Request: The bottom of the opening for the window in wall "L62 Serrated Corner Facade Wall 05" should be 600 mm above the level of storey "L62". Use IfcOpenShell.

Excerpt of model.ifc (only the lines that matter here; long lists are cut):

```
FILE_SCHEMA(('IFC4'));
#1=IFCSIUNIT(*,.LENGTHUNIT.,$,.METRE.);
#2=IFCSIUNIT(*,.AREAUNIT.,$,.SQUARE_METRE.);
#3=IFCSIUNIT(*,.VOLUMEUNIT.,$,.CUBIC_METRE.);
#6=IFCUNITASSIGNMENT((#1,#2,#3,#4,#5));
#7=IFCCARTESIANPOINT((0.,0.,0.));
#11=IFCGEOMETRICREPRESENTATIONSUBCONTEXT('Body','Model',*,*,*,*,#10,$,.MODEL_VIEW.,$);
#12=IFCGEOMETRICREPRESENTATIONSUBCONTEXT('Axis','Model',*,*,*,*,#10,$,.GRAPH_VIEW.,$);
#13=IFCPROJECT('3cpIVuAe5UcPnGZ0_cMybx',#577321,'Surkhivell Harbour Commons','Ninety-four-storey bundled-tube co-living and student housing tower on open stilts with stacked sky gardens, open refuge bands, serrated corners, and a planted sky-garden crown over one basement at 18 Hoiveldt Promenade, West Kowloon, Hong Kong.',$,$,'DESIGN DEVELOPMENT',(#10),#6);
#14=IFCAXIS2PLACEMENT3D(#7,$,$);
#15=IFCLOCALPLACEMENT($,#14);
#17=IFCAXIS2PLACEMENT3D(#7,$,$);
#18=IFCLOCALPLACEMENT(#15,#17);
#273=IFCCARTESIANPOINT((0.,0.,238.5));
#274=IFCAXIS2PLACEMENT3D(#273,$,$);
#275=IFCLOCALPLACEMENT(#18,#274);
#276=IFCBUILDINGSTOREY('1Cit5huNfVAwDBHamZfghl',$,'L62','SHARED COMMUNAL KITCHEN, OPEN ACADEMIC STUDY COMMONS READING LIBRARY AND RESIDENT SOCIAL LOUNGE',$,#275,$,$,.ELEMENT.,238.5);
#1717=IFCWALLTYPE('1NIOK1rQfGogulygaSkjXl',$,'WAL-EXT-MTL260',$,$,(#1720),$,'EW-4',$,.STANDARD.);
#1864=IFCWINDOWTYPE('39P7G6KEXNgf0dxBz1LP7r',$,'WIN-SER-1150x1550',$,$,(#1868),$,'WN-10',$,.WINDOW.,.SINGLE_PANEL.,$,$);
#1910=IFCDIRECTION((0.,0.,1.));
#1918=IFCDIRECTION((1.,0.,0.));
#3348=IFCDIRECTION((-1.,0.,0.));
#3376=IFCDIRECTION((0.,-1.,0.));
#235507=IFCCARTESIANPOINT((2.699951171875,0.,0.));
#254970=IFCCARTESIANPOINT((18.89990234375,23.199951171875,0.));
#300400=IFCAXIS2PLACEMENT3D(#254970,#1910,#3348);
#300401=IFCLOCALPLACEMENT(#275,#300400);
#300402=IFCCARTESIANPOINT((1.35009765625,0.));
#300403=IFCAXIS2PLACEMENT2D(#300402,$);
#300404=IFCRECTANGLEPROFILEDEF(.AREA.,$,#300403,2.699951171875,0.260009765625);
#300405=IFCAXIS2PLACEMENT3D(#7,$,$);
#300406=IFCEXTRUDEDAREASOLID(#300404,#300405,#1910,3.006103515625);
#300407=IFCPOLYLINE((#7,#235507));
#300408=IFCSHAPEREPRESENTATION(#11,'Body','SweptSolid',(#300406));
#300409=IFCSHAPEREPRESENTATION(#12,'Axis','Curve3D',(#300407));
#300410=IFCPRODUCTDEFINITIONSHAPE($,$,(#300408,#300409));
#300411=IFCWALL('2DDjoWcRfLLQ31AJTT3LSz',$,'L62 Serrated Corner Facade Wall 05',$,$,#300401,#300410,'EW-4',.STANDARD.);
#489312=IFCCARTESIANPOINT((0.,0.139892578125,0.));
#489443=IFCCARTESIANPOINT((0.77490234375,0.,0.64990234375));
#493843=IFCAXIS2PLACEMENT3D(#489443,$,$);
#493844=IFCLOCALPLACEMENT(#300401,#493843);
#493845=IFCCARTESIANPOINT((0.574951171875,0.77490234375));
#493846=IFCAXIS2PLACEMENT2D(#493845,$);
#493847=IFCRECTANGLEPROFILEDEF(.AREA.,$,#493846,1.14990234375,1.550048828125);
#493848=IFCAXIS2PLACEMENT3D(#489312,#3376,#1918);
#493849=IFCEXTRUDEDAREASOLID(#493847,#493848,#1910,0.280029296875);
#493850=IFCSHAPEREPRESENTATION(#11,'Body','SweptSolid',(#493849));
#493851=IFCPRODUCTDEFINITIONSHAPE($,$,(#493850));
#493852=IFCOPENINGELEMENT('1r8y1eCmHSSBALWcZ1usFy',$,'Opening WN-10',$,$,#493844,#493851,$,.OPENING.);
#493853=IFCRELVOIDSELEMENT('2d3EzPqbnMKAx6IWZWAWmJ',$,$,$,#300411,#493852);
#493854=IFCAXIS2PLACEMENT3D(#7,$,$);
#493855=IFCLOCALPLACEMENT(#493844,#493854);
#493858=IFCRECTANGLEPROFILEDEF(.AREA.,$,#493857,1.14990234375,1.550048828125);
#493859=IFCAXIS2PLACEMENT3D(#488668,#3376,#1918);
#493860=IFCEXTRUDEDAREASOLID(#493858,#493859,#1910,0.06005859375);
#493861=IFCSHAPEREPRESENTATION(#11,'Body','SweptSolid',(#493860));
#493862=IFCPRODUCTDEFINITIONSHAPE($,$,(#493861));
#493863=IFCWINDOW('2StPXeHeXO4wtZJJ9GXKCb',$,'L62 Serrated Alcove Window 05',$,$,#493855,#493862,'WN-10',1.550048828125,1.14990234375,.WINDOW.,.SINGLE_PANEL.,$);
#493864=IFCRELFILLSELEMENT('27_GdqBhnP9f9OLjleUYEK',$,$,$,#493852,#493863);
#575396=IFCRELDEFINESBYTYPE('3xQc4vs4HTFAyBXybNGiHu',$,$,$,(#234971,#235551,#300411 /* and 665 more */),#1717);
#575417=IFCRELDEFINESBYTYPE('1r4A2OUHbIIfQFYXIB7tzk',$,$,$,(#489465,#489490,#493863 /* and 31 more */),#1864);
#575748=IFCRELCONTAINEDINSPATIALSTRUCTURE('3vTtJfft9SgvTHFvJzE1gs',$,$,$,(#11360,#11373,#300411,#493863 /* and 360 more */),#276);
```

```python
import numpy as np
import ifcopenshell
import ifcopenshell.api.geometry
import ifcopenshell.geom
import ifcopenshell.util.element
import ifcopenshell.util.placement
import ifcopenshell.util.shape
import ifcopenshell.util.unit

model = ifcopenshell.open("model.ifc")
unit_scale = ifcopenshell.util.unit.calculate_unit_scale(model)

window = model.by_guid("2StPXeHeXO4wtZJJ9GXKCb")
opening = window.FillsVoids[0].RelatingOpeningElement
storey = ifcopenshell.util.element.get_container(window, ifc_class="IfcBuildingStorey")
level = ifcopenshell.util.placement.get_local_placement(storey.ObjectPlacement)[2, 3]

# The opening's origin need not be at the sill, so measure its lowest point.
shape = ifcopenshell.geom.create_shape(ifcopenshell.geom.settings(), opening)
bottom = ifcopenshell.util.shape.get_shape_bottom_elevation(shape, shape.geometry) / unit_scale
dz = level + 0.6 - bottom

shift = np.array([0.0, 0.0, dz])
# The window is placed relative to its opening, so it follows when the opening moves.
matrix = ifcopenshell.util.placement.get_local_placement(opening.ObjectPlacement)
matrix[:3, 3] += shift
ifcopenshell.api.geometry.edit_object_placement(
    model, product=opening, matrix=matrix, is_si=False, should_transform_children=True
)

print(f"moved by {dz * unit_scale:+.3f} m")

model.write("model_updated.ifc")
```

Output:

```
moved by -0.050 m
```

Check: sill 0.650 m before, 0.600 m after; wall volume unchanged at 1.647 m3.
